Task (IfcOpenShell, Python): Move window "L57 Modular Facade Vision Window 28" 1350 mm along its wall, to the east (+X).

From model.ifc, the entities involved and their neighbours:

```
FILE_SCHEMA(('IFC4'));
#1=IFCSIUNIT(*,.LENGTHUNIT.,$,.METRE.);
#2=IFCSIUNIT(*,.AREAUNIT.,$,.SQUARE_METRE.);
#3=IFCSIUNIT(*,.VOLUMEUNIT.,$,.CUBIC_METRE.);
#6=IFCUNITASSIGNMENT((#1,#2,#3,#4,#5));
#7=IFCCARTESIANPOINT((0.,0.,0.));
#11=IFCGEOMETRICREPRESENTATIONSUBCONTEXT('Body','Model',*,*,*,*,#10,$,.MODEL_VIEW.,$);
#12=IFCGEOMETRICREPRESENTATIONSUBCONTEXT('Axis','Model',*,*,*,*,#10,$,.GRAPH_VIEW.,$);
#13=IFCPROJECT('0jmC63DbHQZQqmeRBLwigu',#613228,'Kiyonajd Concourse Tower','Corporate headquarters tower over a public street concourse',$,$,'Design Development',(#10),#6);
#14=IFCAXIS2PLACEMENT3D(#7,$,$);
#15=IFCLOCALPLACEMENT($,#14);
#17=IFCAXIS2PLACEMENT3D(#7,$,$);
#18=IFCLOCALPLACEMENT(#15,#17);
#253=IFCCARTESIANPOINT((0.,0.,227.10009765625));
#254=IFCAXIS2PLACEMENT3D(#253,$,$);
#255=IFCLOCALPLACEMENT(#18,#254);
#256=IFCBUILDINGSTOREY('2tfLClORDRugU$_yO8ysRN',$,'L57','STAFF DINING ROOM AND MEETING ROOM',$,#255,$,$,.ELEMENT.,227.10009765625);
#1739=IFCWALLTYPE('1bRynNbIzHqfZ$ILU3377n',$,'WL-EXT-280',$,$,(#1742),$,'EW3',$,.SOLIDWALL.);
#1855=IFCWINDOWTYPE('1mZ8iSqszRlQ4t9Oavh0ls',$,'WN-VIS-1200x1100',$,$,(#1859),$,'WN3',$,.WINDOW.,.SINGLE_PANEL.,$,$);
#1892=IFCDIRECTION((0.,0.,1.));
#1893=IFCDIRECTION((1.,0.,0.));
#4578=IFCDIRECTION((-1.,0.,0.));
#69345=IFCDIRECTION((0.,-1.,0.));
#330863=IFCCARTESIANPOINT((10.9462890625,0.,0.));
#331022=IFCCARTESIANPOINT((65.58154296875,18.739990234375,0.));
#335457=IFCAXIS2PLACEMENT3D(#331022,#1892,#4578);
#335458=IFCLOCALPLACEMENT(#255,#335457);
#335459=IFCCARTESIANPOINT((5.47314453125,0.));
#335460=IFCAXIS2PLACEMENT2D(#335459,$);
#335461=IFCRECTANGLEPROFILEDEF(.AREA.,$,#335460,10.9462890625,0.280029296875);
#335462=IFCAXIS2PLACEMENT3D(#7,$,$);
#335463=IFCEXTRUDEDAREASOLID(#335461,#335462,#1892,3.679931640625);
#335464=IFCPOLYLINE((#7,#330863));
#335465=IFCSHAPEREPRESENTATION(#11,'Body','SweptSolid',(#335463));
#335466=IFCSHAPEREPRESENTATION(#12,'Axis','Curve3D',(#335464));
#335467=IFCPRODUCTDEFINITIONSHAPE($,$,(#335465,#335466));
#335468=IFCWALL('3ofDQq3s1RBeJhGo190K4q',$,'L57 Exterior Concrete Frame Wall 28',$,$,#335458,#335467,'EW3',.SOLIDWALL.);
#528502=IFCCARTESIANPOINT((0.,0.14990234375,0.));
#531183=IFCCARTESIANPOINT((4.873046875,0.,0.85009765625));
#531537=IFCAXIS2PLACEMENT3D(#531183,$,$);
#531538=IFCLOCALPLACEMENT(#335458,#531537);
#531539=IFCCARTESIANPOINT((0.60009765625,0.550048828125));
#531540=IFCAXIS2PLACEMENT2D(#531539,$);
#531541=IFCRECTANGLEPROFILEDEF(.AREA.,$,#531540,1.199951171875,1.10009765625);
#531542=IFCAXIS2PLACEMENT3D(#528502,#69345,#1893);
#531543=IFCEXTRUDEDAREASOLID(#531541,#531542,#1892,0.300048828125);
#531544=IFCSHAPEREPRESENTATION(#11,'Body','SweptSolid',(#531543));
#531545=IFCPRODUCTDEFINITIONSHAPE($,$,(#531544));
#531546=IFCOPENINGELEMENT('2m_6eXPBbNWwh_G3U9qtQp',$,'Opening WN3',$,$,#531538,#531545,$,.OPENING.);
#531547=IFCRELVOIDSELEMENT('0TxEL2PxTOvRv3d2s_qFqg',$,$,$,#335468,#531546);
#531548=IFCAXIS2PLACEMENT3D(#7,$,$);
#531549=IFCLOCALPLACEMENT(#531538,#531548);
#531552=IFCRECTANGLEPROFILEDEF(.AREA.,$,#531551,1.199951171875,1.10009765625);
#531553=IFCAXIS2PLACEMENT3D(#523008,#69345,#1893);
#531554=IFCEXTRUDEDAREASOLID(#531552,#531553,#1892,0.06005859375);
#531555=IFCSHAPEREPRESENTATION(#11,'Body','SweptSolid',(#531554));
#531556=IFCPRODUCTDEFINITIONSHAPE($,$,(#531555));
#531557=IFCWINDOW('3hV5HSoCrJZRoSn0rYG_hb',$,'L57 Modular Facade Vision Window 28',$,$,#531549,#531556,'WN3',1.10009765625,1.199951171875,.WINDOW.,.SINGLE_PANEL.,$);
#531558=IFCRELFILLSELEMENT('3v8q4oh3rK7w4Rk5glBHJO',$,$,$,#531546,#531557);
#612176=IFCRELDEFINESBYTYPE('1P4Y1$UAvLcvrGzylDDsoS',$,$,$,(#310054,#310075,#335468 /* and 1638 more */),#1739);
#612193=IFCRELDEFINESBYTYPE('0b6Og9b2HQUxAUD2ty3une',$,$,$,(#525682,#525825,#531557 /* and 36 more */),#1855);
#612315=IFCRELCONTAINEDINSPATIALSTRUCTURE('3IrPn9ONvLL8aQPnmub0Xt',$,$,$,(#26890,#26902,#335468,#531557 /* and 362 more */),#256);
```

```python
import ifcopenshell
import ifcopenshell.api.geometry
import ifcopenshell.util.placement
import ifcopenshell.util.unit

model = ifcopenshell.open("model.ifc")
unit_scale = ifcopenshell.util.unit.calculate_unit_scale(model)

window = model.by_guid("3hV5HSoCrJZRoSn0rYG_hb")
opening = window.FillsVoids[0].RelatingOpeningElement
wall = opening.VoidsElements[0].RelatingBuildingElement

wall_matrix = ifcopenshell.util.placement.get_local_placement(wall.ObjectPlacement)
shift = wall_matrix[:3, 0] * -1.35 / unit_scale
before = ifcopenshell.util.placement.get_local_placement(window.ObjectPlacement)[:3, 3].copy()

# The window is placed relative to its opening, so it follows when the opening moves.
matrix = ifcopenshell.util.placement.get_local_placement(opening.ObjectPlacement)
matrix[:3, 3] += shift
ifcopenshell.api.geometry.edit_object_placement(
    model, product=opening, matrix=matrix, is_si=False, should_transform_children=True
)

after = ifcopenshell.util.placement.get_local_placement(window.ObjectPlacement)[:3, 3]
print("window moved by", (after - before).round(3) + 0.0)

model.write("model_updated.ifc")
```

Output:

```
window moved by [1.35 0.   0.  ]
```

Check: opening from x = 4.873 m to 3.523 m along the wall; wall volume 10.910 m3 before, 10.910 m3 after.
